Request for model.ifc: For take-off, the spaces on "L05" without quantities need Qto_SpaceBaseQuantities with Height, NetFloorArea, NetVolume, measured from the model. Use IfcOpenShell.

First a look at what the model holds.

```python
import ifcopenshell
import ifcopenshell.util.element
import ifcopenshell.util.unit

model = ifcopenshell.open("model.ifc")
print(model.schema)
for unit_type in ("LENGTHUNIT", "AREAUNIT", "VOLUMEUNIT"):
    print(unit_type, ifcopenshell.util.unit.calculate_unit_scale(model, unit_type))
storey = next(s for s in model.by_type("IfcBuildingStorey") if s.Name == "L05")
spaces = [e for e in ifcopenshell.util.element.get_decomposition(storey) if e.is_a("IfcSpace")]
for e in sorted(spaces, key=lambda e: e.id()):
    print(e.id(), e.is_a(), e.Name, list(ifcopenshell.util.element.get_psets(e, qtos_only=True)), sep=" | ")
```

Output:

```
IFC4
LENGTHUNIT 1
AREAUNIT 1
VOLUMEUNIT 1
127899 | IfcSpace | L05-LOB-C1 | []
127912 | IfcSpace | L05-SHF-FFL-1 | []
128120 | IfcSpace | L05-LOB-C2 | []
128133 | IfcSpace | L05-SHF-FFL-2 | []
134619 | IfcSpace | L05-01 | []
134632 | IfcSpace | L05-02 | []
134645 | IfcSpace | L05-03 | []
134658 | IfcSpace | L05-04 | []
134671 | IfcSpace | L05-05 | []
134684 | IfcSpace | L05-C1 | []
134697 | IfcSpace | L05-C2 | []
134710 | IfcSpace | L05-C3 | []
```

```python
import ifcopenshell
import ifcopenshell.api.pset
import ifcopenshell.geom
import ifcopenshell.util.element
import ifcopenshell.util.shape
import ifcopenshell.util.unit

model = ifcopenshell.open("model.ifc")
unit_scale = ifcopenshell.util.unit.calculate_unit_scale(model)
area_scale = ifcopenshell.util.unit.calculate_unit_scale(model, "AREAUNIT")
volume_scale = ifcopenshell.util.unit.calculate_unit_scale(model, "VOLUMEUNIT")
settings = ifcopenshell.geom.settings()

storey = next(s for s in model.by_type("IfcBuildingStorey") if s.Name == "L05")
spaces = [e for e in ifcopenshell.util.element.get_decomposition(storey) if e.is_a("IfcSpace")]

for e in sorted(spaces, key=lambda e: e.id()):
    if ifcopenshell.util.element.get_psets(e, qtos_only=True, should_inherit=False):
        continue
    # Geometry comes back in metres, in the element's own axes.
    shape = ifcopenshell.geom.create_shape(settings, e)
    values = {
        "Height": ifcopenshell.util.shape.get_z(shape.geometry) / unit_scale,
        "NetFloorArea": ifcopenshell.util.shape.get_footprint_area(shape.geometry) / area_scale,
        "NetVolume": ifcopenshell.util.shape.get_volume(shape.geometry) / volume_scale,
    }
    qto = ifcopenshell.api.pset.add_qto(model, product=e, name="Qto_SpaceBaseQuantities")
    ifcopenshell.api.pset.edit_qto(model, qto=qto, properties=values)
    print(e.id(), {k: round(v, 3) for k, v in values.items()})

model.write("model_edited.ifc")
```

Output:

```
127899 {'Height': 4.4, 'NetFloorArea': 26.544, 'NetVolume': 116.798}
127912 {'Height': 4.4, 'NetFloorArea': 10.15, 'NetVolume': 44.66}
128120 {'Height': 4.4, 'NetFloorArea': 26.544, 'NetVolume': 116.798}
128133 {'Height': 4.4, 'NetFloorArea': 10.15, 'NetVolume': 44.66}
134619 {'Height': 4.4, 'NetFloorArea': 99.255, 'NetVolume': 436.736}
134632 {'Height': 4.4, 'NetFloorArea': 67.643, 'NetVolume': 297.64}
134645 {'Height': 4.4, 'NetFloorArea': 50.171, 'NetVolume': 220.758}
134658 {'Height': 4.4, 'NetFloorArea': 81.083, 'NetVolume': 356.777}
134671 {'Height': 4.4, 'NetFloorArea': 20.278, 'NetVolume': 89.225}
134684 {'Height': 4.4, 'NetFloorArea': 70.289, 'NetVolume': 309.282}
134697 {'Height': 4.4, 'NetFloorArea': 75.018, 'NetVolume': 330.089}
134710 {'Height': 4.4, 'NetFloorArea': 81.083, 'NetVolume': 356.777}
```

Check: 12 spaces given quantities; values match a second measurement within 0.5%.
